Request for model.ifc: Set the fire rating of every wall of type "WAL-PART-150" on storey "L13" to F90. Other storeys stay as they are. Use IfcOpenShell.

First a look at what the model holds.

```python
import ifcopenshell
import ifcopenshell.util.element

model = ifcopenshell.open("model.ifc")
print(model.schema)
storey = next(s for s in model.by_type("IfcBuildingStorey") if s.Name == "L13")
walls = [e for e in ifcopenshell.util.element.get_decomposition(storey) if e.is_a("IfcWall")]
seen = {}
for e in walls:
    element_type = ifcopenshell.util.element.get_type(e)
    key = (element_type.Name if element_type != e and element_type else None, ifcopenshell.util.element.get_pset(e, "Pset_WallCommon", "FireRating"))
    seen[key] = seen.get(key, 0) + 1
for (name, value), count in sorted(seen.items(), key=str):
    print(count, "x", name, "|", value)
```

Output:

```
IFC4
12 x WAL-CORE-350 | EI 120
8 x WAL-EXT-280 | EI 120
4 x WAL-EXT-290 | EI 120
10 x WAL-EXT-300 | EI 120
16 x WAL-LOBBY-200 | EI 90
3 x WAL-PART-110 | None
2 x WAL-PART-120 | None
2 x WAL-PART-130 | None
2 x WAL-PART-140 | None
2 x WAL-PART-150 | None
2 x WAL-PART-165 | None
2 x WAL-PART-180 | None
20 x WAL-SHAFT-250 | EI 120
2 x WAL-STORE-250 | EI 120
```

```python
import ifcopenshell
import ifcopenshell.api.pset
import ifcopenshell.util.element

model = ifcopenshell.open("model.ifc")

storey = next(s for s in model.by_type("IfcBuildingStorey") if s.Name == "L13")
walls = [e for e in ifcopenshell.util.element.get_decomposition(storey) if e.is_a("IfcWall")]

count = 0
for e in walls:
    element_type = ifcopenshell.util.element.get_type(e)
    if element_type in (None, e) or element_type.Name != "WAL-PART-150":
        continue
    # add_pset returns the element's existing set when there is one.
    pset = ifcopenshell.api.pset.add_pset(model, product=e, name="Pset_WallCommon")
    ifcopenshell.api.pset.edit_pset(model, pset=pset, properties={"FireRating": "F90"})
    count += 1

print(count, "walls updated")

model.write("model-out.ifc")
```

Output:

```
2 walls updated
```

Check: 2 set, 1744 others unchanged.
